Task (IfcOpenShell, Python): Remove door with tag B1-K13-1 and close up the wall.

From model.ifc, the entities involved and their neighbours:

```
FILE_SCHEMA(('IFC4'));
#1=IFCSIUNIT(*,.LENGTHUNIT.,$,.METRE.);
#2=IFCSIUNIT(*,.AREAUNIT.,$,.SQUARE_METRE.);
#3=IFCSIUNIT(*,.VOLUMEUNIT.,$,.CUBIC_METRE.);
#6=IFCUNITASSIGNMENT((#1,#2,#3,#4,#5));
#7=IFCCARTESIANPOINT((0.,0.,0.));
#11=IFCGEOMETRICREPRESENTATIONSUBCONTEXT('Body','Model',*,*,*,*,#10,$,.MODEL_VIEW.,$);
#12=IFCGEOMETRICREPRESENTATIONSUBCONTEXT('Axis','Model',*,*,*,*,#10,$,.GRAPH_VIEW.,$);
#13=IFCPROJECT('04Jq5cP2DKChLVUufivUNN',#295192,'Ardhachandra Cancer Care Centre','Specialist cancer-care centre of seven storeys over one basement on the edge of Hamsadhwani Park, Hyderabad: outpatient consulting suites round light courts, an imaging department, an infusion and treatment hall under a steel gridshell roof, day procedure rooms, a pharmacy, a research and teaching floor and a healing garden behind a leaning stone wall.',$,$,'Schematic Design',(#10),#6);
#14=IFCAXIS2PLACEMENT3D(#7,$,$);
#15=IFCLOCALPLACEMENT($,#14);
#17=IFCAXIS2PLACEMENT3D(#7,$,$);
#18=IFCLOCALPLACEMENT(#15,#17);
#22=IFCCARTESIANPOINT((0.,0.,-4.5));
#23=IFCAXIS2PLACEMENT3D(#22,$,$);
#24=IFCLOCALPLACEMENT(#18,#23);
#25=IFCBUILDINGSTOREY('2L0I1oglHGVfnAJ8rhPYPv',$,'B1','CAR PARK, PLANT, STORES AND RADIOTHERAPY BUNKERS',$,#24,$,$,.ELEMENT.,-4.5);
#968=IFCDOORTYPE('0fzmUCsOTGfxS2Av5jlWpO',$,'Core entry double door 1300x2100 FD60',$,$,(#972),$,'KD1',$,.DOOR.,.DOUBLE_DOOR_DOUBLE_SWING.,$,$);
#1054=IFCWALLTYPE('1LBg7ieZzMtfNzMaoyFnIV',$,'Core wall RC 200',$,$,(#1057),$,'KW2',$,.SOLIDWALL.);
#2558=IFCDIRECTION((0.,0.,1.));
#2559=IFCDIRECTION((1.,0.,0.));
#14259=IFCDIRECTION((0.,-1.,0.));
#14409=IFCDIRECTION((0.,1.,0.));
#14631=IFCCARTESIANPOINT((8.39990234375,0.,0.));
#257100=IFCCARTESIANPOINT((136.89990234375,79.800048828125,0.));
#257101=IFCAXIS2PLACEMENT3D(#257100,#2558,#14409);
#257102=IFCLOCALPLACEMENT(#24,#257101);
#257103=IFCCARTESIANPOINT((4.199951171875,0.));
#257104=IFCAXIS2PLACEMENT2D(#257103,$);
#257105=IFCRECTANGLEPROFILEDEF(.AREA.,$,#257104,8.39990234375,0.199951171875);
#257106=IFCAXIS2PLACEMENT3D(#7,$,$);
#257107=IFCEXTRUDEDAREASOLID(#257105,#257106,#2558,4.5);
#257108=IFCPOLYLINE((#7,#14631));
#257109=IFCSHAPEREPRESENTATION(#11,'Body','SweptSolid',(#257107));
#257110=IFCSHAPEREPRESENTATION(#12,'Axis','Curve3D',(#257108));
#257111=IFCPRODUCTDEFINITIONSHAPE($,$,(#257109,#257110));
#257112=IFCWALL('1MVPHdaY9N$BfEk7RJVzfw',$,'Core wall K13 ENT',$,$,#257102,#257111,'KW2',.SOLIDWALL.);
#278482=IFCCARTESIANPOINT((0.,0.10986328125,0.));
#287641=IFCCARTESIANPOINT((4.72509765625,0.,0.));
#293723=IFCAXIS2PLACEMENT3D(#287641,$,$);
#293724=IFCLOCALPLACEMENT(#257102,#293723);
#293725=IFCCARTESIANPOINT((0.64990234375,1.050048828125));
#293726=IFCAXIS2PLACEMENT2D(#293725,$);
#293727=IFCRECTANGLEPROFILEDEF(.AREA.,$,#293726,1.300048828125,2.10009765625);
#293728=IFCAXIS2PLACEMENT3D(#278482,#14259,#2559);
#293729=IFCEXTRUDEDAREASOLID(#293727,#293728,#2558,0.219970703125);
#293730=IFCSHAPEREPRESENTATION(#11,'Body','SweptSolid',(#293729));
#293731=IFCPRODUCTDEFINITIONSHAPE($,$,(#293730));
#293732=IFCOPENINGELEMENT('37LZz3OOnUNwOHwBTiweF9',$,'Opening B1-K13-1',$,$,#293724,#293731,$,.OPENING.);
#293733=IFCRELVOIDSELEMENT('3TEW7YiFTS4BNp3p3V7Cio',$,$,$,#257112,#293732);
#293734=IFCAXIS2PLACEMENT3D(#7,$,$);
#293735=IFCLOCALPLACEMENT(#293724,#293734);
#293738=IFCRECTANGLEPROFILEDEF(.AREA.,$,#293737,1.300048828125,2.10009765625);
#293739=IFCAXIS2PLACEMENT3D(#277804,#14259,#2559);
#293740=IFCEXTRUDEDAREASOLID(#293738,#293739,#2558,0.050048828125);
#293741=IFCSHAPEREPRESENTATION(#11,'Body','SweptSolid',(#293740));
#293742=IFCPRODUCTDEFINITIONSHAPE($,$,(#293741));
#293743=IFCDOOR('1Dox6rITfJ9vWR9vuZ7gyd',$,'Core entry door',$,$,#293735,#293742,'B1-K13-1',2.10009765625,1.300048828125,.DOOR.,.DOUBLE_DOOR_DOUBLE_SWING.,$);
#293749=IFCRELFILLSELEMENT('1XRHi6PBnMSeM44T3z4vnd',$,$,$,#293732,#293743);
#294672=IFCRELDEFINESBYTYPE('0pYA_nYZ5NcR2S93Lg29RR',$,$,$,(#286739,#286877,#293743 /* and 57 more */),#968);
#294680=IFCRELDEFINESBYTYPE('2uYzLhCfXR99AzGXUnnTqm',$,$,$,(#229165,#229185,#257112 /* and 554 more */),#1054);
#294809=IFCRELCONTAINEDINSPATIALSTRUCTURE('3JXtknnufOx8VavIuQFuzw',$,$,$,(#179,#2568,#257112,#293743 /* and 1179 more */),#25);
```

```python
import ifcopenshell
import ifcopenshell.api.feature
import ifcopenshell.api.root
import ifcopenshell.geom
import ifcopenshell.util.shape

model = ifcopenshell.open("model.ifc")
settings = ifcopenshell.geom.settings()


def volume(element):
    """Net volume in cubic metres, openings subtracted."""
    shape = ifcopenshell.geom.create_shape(settings, element)
    return ifcopenshell.util.shape.get_volume(shape.geometry)


door = model.by_guid("1Dox6rITfJ9vWR9vuZ7gyd")
opening = door.FillsVoids[0].RelatingOpeningElement
wall = opening.VoidsElements[0].RelatingBuildingElement
before = volume(wall)

ifcopenshell.api.root.remove_product(model, product=door)
ifcopenshell.api.feature.remove_feature(model, feature=opening)

after = volume(wall)

print(f"wall volume {before:.3f} -> {after:.3f} m3")

model.write("model_rev.ifc")
```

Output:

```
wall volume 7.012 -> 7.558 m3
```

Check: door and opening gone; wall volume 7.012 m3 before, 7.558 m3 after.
